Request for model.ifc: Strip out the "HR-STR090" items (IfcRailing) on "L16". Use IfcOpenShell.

First a look at what the model holds.

```python
import ifcopenshell
import ifcopenshell.util.element

model = ifcopenshell.open("model.ifc")
print(model.schema)
storey = next(s for s in model.by_type("IfcBuildingStorey") if s.Name == "L16")
railings = [e for e in ifcopenshell.util.element.get_decomposition(storey) if e.is_a("IfcRailing")]
seen = {}
for e in railings:
    element_type = ifcopenshell.util.element.get_type(e)
    name = element_type.Name if element_type not in (None, e) else None
    seen[name] = seen.get(name, 0) + 1
for name, count in sorted(seen.items(), key=str):
    print(count, "x", name)
```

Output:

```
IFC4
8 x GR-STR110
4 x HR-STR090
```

```python
import ifcopenshell
import ifcopenshell.api.root
import ifcopenshell.util.element

model = ifcopenshell.open("model.ifc")

storey = next(s for s in model.by_type("IfcBuildingStorey") if s.Name == "L16")
railings = [e for e in ifcopenshell.util.element.get_decomposition(storey) if e.is_a("IfcRailing")]
targets = [e for e in railings if (t := ifcopenshell.util.element.get_type(e)) not in (None, e) and t.Name == "HR-STR090"]

for e in targets:
    ifcopenshell.api.root.remove_product(model, product=e)
print(len(targets), "removed")

model.write("model_updated.ifc")
```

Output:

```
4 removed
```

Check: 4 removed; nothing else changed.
